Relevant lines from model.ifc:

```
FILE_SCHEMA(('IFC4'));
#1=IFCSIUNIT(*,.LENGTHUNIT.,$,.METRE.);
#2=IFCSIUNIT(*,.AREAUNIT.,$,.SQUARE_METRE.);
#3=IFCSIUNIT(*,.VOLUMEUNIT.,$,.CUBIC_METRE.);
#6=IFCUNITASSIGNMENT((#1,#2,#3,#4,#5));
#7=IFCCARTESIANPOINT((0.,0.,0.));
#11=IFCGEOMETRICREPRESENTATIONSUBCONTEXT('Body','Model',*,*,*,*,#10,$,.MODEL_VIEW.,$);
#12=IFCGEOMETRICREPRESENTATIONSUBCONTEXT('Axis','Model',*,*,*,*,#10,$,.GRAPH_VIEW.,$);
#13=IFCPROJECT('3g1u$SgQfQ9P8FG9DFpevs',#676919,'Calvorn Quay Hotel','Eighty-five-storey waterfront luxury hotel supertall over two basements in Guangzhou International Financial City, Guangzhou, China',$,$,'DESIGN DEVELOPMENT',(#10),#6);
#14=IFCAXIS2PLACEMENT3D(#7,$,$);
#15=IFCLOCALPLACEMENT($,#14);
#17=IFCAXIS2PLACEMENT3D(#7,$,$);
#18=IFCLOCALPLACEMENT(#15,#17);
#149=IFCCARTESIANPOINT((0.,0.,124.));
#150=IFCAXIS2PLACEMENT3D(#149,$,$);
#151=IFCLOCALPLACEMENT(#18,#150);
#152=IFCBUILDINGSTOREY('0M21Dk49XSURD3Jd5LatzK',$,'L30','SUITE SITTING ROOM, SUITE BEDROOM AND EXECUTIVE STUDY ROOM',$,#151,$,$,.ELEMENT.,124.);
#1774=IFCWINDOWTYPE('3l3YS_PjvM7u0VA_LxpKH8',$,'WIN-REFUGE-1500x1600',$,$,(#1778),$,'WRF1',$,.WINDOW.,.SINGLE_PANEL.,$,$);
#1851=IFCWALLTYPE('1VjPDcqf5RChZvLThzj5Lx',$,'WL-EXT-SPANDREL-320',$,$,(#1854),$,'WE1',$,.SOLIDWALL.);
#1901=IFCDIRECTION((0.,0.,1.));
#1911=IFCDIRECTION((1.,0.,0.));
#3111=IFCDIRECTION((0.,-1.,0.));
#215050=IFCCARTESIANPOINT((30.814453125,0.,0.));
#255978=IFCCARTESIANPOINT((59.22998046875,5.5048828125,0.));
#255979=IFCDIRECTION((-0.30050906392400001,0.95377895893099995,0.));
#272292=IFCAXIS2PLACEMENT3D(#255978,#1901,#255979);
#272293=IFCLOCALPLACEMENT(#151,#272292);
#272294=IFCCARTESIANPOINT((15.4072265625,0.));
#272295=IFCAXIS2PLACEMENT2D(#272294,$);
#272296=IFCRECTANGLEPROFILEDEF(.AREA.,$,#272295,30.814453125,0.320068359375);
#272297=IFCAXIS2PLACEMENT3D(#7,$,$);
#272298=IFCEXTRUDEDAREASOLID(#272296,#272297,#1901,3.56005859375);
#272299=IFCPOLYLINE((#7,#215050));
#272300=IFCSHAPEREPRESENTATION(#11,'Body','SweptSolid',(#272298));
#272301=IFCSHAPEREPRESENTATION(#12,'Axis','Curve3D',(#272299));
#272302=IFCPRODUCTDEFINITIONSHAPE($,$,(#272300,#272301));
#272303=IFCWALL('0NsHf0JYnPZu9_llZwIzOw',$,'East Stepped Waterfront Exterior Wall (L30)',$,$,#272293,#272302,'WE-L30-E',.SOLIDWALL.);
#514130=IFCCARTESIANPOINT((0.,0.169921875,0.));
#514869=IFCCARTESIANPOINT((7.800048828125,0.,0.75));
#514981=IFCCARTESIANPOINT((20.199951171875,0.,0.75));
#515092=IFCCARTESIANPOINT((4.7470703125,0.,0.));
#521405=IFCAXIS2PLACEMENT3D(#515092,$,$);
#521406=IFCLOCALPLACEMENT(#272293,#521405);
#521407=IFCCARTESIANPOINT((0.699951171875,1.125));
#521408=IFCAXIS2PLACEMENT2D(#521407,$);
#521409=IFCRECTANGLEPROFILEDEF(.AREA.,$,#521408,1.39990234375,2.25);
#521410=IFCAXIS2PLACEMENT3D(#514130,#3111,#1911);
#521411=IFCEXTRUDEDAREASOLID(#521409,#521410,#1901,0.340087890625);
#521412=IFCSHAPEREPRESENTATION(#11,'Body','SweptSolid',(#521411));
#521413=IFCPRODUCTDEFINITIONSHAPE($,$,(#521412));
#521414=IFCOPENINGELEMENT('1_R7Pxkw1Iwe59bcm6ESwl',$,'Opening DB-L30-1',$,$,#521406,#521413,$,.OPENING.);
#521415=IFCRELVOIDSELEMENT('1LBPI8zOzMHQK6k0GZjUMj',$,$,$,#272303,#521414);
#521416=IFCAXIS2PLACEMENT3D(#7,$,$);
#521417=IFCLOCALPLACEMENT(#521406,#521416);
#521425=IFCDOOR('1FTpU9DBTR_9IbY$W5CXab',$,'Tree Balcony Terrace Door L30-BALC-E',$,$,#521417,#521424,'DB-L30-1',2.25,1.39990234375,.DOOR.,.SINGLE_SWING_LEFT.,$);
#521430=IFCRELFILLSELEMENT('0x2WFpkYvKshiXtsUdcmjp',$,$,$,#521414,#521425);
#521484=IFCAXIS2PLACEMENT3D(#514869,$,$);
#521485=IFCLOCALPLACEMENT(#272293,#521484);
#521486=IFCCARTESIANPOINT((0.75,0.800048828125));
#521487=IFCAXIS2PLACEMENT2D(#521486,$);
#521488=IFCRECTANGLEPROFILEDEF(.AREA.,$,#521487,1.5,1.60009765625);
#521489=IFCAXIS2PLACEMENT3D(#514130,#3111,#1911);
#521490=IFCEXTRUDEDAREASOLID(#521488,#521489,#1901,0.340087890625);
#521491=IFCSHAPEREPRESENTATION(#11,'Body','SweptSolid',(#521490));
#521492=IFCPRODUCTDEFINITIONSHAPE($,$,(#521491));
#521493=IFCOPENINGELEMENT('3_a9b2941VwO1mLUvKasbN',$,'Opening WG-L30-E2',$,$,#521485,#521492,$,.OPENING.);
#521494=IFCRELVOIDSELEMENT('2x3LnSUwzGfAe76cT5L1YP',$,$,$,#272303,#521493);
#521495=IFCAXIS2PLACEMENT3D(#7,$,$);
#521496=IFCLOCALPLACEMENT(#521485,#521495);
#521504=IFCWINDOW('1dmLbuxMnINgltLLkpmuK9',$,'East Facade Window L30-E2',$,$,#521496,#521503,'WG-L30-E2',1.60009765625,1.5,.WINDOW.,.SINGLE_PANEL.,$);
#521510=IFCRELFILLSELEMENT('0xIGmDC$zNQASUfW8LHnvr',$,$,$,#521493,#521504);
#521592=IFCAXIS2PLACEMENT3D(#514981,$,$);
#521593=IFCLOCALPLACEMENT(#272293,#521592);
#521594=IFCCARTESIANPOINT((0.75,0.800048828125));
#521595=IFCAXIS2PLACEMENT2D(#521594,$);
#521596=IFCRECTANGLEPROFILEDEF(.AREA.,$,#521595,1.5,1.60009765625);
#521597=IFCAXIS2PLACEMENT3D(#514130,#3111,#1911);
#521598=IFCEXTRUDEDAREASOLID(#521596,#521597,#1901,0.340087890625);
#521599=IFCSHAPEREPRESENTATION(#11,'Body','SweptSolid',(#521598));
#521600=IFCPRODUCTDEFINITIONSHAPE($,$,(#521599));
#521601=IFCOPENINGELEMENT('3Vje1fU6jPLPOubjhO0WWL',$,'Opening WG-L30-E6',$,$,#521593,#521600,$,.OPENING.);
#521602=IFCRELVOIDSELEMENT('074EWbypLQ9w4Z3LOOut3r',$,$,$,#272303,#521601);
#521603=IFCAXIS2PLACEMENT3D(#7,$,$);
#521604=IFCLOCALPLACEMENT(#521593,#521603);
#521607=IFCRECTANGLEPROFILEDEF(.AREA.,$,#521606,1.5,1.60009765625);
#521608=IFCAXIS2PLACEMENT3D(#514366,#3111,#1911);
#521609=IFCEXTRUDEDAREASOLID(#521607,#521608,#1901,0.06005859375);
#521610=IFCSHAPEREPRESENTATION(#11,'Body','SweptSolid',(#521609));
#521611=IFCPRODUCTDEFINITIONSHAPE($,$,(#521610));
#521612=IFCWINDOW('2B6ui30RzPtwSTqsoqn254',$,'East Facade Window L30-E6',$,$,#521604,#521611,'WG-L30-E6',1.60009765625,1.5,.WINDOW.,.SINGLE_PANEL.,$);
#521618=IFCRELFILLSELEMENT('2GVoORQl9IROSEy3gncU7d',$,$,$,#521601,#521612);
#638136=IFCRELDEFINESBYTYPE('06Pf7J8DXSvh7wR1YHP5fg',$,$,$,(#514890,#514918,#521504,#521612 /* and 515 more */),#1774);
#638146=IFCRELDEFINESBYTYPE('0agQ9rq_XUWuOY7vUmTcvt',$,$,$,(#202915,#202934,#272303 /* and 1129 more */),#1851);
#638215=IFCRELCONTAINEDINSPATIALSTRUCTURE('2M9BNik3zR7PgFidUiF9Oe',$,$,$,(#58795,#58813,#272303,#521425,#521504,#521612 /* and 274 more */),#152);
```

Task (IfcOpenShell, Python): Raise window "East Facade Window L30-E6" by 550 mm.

```python
import numpy as np
import ifcopenshell
import ifcopenshell.api.geometry
import ifcopenshell.util.placement
import ifcopenshell.util.unit

model = ifcopenshell.open("model.ifc")
unit_scale = ifcopenshell.util.unit.calculate_unit_scale(model)

window = model.by_id(521612)
opening = window.FillsVoids[0].RelatingOpeningElement
dz = 0.55 / unit_scale

shift = np.array([0.0, 0.0, dz])
# The window is placed relative to its opening, so it follows when the opening moves.
matrix = ifcopenshell.util.placement.get_local_placement(opening.ObjectPlacement)
matrix[:3, 3] += shift
ifcopenshell.api.geometry.edit_object_placement(
    model, product=opening, matrix=matrix, is_si=False, should_transform_children=True
)

print(f"moved by {dz * unit_scale:+.3f} m")

model.write("model_rev.ifc")
```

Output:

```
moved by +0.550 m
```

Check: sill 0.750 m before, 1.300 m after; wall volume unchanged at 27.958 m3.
